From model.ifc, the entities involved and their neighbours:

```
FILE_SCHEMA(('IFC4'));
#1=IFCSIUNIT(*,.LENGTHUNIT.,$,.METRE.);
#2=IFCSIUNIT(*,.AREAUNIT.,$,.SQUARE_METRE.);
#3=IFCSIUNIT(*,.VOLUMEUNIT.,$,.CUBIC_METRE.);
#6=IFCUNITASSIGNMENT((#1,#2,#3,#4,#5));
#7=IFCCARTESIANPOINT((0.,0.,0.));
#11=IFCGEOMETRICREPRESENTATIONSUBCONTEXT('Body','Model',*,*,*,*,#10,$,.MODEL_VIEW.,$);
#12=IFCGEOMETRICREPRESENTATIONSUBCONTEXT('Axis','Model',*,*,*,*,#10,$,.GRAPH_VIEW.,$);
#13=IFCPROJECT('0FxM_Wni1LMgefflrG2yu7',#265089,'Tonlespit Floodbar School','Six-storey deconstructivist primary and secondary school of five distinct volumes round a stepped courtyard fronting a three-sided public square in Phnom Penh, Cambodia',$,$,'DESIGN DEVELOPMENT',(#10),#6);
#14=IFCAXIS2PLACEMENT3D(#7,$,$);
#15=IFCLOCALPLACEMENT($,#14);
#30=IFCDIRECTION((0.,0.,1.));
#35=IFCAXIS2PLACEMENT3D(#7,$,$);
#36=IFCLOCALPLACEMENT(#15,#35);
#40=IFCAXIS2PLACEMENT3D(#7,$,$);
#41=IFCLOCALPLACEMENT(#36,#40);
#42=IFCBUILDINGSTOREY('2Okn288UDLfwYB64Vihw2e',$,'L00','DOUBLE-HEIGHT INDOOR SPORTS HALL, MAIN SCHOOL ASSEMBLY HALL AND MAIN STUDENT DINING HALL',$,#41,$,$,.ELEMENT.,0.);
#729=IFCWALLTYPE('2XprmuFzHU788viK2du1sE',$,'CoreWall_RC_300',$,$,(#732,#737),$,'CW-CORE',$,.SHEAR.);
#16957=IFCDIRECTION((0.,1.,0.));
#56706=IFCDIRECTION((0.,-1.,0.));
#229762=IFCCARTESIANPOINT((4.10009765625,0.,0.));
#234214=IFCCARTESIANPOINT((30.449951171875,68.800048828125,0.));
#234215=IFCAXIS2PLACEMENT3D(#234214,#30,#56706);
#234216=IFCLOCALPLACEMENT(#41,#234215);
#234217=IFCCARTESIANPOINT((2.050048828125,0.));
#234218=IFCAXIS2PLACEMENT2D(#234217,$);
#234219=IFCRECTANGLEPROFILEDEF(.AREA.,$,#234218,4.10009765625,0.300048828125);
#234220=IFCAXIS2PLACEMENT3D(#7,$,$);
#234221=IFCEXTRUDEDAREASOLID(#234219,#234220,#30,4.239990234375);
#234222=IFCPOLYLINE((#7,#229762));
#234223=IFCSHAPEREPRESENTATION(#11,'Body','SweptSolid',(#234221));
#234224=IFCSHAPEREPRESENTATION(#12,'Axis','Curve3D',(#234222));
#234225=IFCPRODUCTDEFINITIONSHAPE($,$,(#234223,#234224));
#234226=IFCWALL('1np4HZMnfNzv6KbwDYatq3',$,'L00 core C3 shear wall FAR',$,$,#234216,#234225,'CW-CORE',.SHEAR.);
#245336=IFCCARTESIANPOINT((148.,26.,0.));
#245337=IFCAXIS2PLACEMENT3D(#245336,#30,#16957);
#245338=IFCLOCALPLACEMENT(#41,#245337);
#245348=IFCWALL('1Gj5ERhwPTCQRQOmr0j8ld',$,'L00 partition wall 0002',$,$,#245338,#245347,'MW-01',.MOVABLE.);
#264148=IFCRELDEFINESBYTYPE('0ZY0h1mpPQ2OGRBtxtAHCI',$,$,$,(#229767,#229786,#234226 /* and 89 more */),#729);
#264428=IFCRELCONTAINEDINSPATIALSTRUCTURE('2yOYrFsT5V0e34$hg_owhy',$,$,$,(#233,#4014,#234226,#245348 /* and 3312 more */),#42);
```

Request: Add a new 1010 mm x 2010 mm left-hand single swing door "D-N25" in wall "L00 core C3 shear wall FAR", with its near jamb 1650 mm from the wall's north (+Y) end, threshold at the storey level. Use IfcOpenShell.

```python
import numpy as np
import ifcopenshell
import ifcopenshell.api.feature
import ifcopenshell.api.geometry
import ifcopenshell.api.root
import ifcopenshell.api.spatial
import ifcopenshell.geom
import ifcopenshell.util.element
import ifcopenshell.util.placement
import ifcopenshell.util.representation
import ifcopenshell.util.shape
import ifcopenshell.util.unit

model = ifcopenshell.open("model.ifc")
unit_scale = ifcopenshell.util.unit.calculate_unit_scale(model)
settings = ifcopenshell.geom.settings()


def volume(element):
    """Net volume in cubic metres, openings subtracted."""
    shape = ifcopenshell.geom.create_shape(settings, element)
    return ifcopenshell.util.shape.get_volume(shape.geometry)


wall = model.by_guid("1np4HZMnfNzv6KbwDYatq3")
storey = ifcopenshell.util.element.get_container(wall, ifc_class="IfcBuildingStorey")
context = ifcopenshell.util.representation.get_context(model, "Model", "Body", "MODEL_VIEW")
before = volume(wall)

width, height, from_end, sill = 1.01, 2.01, 1.65, 0.0  # metres

# The wall runs along its own X axis, and the end named is its -X end.
wall_shape = ifcopenshell.geom.create_shape(settings, wall)
x, y, z = ifcopenshell.util.shape.get_vertices(wall_shape.geometry).T
start = x.min() + from_end
face, thickness = float(y.min()), float(y.max() - y.min())
wall_matrix = ifcopenshell.util.placement.get_local_placement(wall.ObjectPlacement)
level = ifcopenshell.util.placement.get_local_placement(storey.ObjectPlacement)[2, 3]


def in_wall(x, y):
    """Placement at x, y metres in the wall's axes, at sill height."""
    matrix = wall_matrix.copy()
    matrix[:, 3] = wall_matrix @ np.array([x / unit_scale, y / unit_scale, 0.0, 1.0])
    matrix[2, 3] = level + sill / unit_scale
    return matrix


# Opening: a box that overshoots both wall faces by 50 mm.
opening = ifcopenshell.api.root.create_entity(model, ifc_class="IfcOpeningElement", predefined_type="OPENING")
box = ifcopenshell.api.geometry.add_wall_representation(
    model, context=context, length=width, height=height, thickness=thickness + 0.1
)
ifcopenshell.api.geometry.assign_representation(model, product=opening, representation=box)
ifcopenshell.api.geometry.edit_object_placement(model, product=opening, matrix=in_wall(start, face - 0.05), is_si=False)
ifcopenshell.api.feature.add_feature(model, feature=opening, element=wall)

door = ifcopenshell.api.root.create_entity(model, ifc_class="IfcDoor", name="D-N25", predefined_type="DOOR")
door.OverallWidth, door.OverallHeight = width / unit_scale, height / unit_scale
door.OperationType = "SINGLE_SWING_LEFT"
body = ifcopenshell.api.geometry.add_door_representation(
    model,
    context=context,
    overall_width=door.OverallWidth,
    overall_height=door.OverallHeight,
    operation_type="SINGLE_SWING_LEFT",
    lining_properties={"LiningDepth": thickness / unit_scale, "ThresholdDepth": thickness / unit_scale},
)
ifcopenshell.api.geometry.assign_representation(model, product=door, representation=body)
ifcopenshell.api.spatial.assign_container(model, products=[door], relating_structure=storey)
ifcopenshell.api.feature.add_filling(model, opening=opening, element=door)

# The lining spans the wall, so the door starts at the wall face.
ifcopenshell.api.geometry.edit_object_placement(model, product=door, matrix=in_wall(start, face), is_si=False)

after = volume(wall)

print(f"wall volume {before:.3f} -> {after:.3f} m3")

model.write("model_edited.ifc")
```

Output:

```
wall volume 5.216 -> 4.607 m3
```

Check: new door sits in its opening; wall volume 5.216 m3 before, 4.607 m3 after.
